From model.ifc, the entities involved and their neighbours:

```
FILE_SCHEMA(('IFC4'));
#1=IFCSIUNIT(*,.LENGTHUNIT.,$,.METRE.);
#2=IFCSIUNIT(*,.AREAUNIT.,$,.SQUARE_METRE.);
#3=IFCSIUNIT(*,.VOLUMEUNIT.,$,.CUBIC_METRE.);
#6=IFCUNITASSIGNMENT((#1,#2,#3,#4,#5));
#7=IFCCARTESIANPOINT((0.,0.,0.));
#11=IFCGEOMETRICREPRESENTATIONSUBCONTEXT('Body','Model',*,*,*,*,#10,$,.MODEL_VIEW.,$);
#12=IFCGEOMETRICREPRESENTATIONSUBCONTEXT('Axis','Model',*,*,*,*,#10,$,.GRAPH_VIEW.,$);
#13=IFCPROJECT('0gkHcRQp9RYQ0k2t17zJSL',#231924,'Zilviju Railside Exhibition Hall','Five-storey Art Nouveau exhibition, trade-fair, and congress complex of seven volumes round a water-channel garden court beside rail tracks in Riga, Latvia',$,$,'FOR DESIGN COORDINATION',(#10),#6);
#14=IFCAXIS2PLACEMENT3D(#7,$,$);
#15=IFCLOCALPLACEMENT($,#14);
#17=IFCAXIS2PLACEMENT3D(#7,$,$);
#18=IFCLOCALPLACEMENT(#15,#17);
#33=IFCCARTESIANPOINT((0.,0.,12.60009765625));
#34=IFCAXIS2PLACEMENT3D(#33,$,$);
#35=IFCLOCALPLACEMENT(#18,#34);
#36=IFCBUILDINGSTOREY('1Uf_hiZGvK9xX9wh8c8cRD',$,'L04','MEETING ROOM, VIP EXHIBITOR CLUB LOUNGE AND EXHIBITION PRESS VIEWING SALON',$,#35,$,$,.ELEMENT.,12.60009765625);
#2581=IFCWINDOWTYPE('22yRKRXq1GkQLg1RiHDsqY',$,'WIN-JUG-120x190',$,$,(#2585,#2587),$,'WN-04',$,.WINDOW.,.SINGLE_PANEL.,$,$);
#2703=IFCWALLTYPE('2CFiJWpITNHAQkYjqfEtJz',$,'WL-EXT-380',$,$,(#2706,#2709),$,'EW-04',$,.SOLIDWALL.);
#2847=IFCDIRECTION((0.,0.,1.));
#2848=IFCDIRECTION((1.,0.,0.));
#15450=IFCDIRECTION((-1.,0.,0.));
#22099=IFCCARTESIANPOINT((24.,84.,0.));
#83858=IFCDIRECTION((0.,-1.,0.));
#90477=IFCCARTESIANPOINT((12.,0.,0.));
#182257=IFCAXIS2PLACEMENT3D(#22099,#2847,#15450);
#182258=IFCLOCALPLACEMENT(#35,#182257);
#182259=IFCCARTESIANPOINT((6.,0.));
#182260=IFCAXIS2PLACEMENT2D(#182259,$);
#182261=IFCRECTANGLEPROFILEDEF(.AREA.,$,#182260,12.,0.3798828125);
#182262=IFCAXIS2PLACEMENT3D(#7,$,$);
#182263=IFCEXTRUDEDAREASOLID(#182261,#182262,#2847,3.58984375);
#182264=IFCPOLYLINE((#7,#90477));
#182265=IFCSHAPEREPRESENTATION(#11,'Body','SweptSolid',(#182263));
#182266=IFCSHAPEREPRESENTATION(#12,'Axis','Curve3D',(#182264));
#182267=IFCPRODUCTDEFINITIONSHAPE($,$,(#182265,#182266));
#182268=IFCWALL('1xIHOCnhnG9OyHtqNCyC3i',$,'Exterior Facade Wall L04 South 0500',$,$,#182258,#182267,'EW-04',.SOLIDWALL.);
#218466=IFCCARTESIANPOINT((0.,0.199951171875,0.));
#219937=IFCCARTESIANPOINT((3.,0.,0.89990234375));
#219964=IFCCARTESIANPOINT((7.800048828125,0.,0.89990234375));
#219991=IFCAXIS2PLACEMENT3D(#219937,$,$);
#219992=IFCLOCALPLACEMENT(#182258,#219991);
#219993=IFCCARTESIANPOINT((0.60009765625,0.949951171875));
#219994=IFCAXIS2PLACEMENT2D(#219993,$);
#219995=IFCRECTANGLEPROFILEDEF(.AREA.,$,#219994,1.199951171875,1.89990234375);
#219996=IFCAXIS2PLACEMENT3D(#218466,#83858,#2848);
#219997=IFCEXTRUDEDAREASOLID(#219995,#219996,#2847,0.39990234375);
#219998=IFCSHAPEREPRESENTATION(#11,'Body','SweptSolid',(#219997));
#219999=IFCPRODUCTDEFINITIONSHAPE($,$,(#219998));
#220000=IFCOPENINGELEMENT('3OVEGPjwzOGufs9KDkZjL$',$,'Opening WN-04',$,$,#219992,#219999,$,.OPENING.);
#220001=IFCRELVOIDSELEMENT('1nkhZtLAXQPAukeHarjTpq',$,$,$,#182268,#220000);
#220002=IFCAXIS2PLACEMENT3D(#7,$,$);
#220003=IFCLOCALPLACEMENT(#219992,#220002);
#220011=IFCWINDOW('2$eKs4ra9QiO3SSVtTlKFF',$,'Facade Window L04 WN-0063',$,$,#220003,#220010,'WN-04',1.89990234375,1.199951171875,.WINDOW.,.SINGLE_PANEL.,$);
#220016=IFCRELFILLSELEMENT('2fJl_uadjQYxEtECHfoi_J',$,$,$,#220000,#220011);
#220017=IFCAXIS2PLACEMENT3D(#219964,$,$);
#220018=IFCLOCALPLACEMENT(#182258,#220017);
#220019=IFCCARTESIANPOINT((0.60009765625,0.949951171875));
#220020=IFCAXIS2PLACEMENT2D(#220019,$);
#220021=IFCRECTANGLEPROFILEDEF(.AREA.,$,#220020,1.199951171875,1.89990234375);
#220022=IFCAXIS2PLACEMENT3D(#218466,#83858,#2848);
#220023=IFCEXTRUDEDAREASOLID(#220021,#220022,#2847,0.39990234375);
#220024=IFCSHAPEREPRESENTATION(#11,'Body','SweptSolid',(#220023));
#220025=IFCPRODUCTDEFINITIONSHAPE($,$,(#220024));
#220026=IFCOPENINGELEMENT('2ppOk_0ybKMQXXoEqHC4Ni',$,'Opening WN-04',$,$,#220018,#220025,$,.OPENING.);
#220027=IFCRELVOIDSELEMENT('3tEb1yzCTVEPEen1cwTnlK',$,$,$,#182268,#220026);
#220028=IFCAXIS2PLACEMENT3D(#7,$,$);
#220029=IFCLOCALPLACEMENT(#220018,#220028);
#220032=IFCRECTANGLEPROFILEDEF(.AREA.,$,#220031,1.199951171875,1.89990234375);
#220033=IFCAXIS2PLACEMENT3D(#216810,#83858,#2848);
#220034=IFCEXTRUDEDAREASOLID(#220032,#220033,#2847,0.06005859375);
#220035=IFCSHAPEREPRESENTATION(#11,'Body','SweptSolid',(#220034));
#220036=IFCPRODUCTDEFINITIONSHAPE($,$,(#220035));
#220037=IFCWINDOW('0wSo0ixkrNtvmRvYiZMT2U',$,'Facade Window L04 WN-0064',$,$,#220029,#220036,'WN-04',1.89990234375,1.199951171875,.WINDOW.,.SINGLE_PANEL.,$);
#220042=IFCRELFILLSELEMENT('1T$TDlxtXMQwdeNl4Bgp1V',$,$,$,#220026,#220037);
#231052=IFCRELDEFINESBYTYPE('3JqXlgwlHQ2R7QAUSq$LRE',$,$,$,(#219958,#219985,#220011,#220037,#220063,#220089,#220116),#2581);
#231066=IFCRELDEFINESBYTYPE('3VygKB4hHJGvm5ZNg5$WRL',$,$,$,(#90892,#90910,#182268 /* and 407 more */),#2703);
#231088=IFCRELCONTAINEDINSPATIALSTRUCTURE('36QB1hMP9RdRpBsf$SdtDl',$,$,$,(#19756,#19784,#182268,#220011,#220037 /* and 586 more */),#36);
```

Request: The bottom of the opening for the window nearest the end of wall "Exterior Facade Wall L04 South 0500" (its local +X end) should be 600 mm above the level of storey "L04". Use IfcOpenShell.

```python
import numpy as np
import ifcopenshell
import ifcopenshell.api.geometry
import ifcopenshell.geom
import ifcopenshell.util.element
import ifcopenshell.util.placement
import ifcopenshell.util.shape
import ifcopenshell.util.unit

model = ifcopenshell.open("model.ifc")
unit_scale = ifcopenshell.util.unit.calculate_unit_scale(model)

window = model.by_id(220037)
opening = window.FillsVoids[0].RelatingOpeningElement
storey = ifcopenshell.util.element.get_container(window, ifc_class="IfcBuildingStorey")
level = ifcopenshell.util.placement.get_local_placement(storey.ObjectPlacement)[2, 3]

# The opening's origin need not be at the sill, so measure its lowest point.
shape = ifcopenshell.geom.create_shape(ifcopenshell.geom.settings(), opening)
bottom = ifcopenshell.util.shape.get_shape_bottom_elevation(shape, shape.geometry) / unit_scale
dz = level + 0.6 / unit_scale - bottom

shift = np.array([0.0, 0.0, dz])
# The window is placed relative to its opening, so it follows when the opening moves.
matrix = ifcopenshell.util.placement.get_local_placement(opening.ObjectPlacement)
matrix[:3, 3] += shift
ifcopenshell.api.geometry.edit_object_placement(
    model, product=opening, matrix=matrix, is_si=False, should_transform_children=True
)

print(f"moved by {dz * unit_scale:+.3f} m")

model.write("model_edited.ifc")
```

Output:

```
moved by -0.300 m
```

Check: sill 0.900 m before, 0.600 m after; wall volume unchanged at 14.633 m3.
